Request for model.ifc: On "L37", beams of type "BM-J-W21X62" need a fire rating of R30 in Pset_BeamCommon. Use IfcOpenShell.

First a look at what the model holds.

```python
import ifcopenshell
import ifcopenshell.util.element

model = ifcopenshell.open("model.ifc")
print(model.schema)
storey = next(s for s in model.by_type("IfcBuildingStorey") if s.Name == "L37")
beams = [e for e in ifcopenshell.util.element.get_decomposition(storey) if e.is_a("IfcBeam")]
seen = {}
for e in beams:
    element_type = ifcopenshell.util.element.get_type(e)
    key = (element_type.Name if element_type != e and element_type else None, ifcopenshell.util.element.get_pset(e, "Pset_BeamCommon", "FireRating"))
    seen[key] = seen.get(key, 0) + 1
for (name, value), count in sorted(seen.items(), key=str):
    print(count, "x", name, "|", value)
```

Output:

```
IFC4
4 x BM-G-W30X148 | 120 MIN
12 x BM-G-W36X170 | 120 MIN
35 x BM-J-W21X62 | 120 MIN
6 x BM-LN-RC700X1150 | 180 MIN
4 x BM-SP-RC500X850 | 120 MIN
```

```python
import ifcopenshell
import ifcopenshell.api.pset
import ifcopenshell.util.element

model = ifcopenshell.open("model.ifc")

storey = next(s for s in model.by_type("IfcBuildingStorey") if s.Name == "L37")
beams = [e for e in ifcopenshell.util.element.get_decomposition(storey) if e.is_a("IfcBeam")]

count = 0
for e in beams:
    element_type = ifcopenshell.util.element.get_type(e)
    if element_type in (None, e) or element_type.Name != "BM-J-W21X62":
        continue
    found = ifcopenshell.util.element.get_pset(e, "Pset_BeamCommon", should_inherit=False)
    if found:
        pset = model.by_id(found["id"])
        if len(ifcopenshell.util.element.get_elements_by_pset(pset)) > 1:
            pset = ifcopenshell.api.pset.unshare_pset(model, products=[e], pset=pset)[0]
    else:
        pset = ifcopenshell.api.pset.add_pset(model, product=e, name="Pset_BeamCommon")
    ifcopenshell.api.pset.edit_pset(model, pset=pset, properties={"FireRating": "R30"})
    count += 1

print(count, "beams updated")

model.write("model_updated.ifc")
```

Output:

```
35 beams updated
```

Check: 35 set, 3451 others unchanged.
